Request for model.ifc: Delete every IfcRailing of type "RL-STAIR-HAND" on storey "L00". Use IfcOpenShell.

First a look at what the model holds.

```python
import ifcopenshell
import ifcopenshell.util.element

model = ifcopenshell.open("model.ifc")
print(model.schema)
storey = next(s for s in model.by_type("IfcBuildingStorey") if s.Name == "L00")
railings = [e for e in ifcopenshell.util.element.get_decomposition(storey) if e.is_a("IfcRailing")]
seen = {}
for e in railings:
    element_type = ifcopenshell.util.element.get_type(e)
    name = element_type.Name if element_type not in (None, e) else None
    seen[name] = seen.get(name, 0) + 1
for name, count in sorted(seen.items(), key=str):
    print(count, "x", name)
```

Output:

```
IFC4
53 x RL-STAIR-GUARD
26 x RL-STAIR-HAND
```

```python
import ifcopenshell
import ifcopenshell.api.root
import ifcopenshell.util.element

model = ifcopenshell.open("model.ifc")

storey = next(s for s in model.by_type("IfcBuildingStorey") if s.Name == "L00")
railings = [e for e in ifcopenshell.util.element.get_decomposition(storey) if e.is_a("IfcRailing")]
targets = [e for e in railings if (t := ifcopenshell.util.element.get_type(e)) not in (None, e) and t.Name == "RL-STAIR-HAND"]

for e in targets:
    ifcopenshell.api.root.remove_product(model, product=e)
print(len(targets), "removed")

model.write("model_edited.ifc")
```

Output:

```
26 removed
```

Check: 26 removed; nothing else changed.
